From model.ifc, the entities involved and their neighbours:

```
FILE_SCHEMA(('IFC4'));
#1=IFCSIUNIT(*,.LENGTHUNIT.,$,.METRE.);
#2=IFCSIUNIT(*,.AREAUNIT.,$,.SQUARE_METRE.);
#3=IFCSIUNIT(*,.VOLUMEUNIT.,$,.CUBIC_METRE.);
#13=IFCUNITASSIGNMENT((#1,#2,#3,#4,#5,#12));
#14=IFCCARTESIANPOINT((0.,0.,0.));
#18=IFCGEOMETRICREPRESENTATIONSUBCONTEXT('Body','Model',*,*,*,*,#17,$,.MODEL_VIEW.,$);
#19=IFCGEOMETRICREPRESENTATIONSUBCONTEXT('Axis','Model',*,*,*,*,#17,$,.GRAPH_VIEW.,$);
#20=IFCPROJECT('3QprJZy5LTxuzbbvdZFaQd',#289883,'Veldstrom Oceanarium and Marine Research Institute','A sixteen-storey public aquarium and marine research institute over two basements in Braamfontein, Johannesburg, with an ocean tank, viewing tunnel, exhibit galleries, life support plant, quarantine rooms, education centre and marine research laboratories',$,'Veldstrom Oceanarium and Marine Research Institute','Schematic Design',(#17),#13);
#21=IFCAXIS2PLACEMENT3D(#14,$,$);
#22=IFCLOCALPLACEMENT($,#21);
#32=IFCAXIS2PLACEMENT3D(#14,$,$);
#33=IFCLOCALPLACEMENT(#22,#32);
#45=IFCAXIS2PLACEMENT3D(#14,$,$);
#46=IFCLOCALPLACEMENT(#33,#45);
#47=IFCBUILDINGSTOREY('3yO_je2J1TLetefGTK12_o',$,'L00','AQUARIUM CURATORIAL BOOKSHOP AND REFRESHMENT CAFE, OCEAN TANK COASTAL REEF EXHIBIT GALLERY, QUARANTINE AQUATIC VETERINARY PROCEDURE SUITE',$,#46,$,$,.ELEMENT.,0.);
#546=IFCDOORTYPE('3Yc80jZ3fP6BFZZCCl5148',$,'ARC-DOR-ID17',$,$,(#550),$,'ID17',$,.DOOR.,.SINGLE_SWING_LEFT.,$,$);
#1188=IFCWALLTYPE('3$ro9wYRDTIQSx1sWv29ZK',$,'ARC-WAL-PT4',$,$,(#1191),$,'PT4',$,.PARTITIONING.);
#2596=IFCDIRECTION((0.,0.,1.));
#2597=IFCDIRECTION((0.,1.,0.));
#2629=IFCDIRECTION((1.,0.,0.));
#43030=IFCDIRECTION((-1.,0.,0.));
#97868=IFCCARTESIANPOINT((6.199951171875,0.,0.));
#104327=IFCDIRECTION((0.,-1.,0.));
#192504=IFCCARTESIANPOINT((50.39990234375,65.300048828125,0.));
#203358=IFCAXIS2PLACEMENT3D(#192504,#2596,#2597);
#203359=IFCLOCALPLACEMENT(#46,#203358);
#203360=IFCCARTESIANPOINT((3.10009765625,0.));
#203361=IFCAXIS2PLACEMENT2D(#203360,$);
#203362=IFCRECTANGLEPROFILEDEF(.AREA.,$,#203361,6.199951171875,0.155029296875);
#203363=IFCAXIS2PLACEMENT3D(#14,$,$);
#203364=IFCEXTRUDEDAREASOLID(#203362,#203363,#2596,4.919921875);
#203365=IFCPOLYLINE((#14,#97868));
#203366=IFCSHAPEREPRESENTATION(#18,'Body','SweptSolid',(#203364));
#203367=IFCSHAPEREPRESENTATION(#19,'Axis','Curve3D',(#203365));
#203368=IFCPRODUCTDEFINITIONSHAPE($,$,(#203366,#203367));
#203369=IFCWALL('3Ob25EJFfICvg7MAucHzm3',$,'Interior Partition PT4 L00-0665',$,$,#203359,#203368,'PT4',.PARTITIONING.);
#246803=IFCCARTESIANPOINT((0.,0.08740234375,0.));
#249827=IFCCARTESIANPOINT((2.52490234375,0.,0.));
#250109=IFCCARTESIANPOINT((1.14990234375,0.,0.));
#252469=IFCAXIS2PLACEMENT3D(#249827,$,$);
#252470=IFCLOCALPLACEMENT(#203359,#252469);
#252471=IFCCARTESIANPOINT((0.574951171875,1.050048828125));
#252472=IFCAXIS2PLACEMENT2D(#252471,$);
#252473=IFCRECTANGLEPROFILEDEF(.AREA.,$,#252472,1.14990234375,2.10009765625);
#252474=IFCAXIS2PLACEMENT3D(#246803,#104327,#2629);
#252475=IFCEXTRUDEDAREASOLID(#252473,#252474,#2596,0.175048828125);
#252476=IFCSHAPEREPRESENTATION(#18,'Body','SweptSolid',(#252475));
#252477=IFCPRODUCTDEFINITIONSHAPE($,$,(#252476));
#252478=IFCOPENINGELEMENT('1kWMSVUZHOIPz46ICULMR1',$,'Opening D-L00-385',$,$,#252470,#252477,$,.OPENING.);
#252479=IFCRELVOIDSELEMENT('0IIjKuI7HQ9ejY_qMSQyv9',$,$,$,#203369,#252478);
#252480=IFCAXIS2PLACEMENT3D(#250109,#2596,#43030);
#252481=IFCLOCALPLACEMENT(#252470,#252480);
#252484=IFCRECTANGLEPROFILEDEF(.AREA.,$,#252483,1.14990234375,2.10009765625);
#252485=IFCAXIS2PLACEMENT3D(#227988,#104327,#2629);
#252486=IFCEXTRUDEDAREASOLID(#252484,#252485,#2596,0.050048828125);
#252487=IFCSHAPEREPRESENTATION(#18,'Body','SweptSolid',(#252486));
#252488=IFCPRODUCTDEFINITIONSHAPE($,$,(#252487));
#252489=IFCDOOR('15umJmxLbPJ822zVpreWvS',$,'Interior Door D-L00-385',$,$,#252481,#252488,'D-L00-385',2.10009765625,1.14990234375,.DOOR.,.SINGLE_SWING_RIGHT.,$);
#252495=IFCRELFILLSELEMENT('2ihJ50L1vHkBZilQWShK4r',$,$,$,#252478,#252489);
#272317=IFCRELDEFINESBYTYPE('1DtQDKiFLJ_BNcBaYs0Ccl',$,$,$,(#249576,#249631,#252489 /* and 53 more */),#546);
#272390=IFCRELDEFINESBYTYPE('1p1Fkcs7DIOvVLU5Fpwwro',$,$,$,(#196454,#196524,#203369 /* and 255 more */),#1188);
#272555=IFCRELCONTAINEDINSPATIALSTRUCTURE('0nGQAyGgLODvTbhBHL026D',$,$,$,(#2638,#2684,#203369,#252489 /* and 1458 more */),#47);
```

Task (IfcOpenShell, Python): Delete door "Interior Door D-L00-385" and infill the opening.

```python
import ifcopenshell
import ifcopenshell.api.feature
import ifcopenshell.api.root
import ifcopenshell.geom
import ifcopenshell.util.shape

model = ifcopenshell.open("model.ifc")
settings = ifcopenshell.geom.settings()


def volume(element):
    """Net volume in cubic metres, openings subtracted."""
    shape = ifcopenshell.geom.create_shape(settings, element)
    return ifcopenshell.util.shape.get_volume(shape.geometry)


door = model.by_guid("15umJmxLbPJ822zVpreWvS")
opening = door.FillsVoids[0].RelatingOpeningElement
wall = opening.VoidsElements[0].RelatingBuildingElement
before = volume(wall)

ifcopenshell.api.root.remove_product(model, product=door)
ifcopenshell.api.feature.remove_feature(model, feature=opening)

after = volume(wall)

print(f"wall volume {before:.3f} -> {after:.3f} m3")

model.write("model_v2.ifc")
```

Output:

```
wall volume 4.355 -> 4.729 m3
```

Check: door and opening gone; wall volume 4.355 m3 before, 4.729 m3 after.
